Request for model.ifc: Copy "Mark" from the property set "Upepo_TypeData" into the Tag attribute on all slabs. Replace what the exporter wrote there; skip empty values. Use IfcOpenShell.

First a look at what the model holds.

```python
import ifcopenshell
import ifcopenshell.util.element

model = ifcopenshell.open("model.ifc")
print(model.schema)
slabs = model.by_type("IfcSlab")
print(len(slabs), "slabs")
for e in slabs[:8]:
    source = ifcopenshell.util.element.get_pset(e, "Upepo_TypeData", "Mark")
    target = e.Tag
    print(e.id(), repr(source), repr(target), sep=" | ")
```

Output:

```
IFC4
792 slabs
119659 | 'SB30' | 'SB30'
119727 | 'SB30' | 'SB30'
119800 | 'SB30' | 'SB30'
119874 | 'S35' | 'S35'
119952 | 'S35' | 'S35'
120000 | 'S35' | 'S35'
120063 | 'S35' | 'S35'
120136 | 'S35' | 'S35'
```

```python
import ifcopenshell
import ifcopenshell.util.element

model = ifcopenshell.open("model.ifc")

count = 0
for e in model.by_type("IfcSlab"):
    value = ifcopenshell.util.element.get_pset(e, "Upepo_TypeData", "Mark")
    current = e.Tag
    if not value or not value.strip() or current == value:
        continue
    e.Tag = value
    count += 1

print(count, "slabs updated")

model.write("model-out.ifc")
```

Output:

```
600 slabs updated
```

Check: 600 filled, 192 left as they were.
